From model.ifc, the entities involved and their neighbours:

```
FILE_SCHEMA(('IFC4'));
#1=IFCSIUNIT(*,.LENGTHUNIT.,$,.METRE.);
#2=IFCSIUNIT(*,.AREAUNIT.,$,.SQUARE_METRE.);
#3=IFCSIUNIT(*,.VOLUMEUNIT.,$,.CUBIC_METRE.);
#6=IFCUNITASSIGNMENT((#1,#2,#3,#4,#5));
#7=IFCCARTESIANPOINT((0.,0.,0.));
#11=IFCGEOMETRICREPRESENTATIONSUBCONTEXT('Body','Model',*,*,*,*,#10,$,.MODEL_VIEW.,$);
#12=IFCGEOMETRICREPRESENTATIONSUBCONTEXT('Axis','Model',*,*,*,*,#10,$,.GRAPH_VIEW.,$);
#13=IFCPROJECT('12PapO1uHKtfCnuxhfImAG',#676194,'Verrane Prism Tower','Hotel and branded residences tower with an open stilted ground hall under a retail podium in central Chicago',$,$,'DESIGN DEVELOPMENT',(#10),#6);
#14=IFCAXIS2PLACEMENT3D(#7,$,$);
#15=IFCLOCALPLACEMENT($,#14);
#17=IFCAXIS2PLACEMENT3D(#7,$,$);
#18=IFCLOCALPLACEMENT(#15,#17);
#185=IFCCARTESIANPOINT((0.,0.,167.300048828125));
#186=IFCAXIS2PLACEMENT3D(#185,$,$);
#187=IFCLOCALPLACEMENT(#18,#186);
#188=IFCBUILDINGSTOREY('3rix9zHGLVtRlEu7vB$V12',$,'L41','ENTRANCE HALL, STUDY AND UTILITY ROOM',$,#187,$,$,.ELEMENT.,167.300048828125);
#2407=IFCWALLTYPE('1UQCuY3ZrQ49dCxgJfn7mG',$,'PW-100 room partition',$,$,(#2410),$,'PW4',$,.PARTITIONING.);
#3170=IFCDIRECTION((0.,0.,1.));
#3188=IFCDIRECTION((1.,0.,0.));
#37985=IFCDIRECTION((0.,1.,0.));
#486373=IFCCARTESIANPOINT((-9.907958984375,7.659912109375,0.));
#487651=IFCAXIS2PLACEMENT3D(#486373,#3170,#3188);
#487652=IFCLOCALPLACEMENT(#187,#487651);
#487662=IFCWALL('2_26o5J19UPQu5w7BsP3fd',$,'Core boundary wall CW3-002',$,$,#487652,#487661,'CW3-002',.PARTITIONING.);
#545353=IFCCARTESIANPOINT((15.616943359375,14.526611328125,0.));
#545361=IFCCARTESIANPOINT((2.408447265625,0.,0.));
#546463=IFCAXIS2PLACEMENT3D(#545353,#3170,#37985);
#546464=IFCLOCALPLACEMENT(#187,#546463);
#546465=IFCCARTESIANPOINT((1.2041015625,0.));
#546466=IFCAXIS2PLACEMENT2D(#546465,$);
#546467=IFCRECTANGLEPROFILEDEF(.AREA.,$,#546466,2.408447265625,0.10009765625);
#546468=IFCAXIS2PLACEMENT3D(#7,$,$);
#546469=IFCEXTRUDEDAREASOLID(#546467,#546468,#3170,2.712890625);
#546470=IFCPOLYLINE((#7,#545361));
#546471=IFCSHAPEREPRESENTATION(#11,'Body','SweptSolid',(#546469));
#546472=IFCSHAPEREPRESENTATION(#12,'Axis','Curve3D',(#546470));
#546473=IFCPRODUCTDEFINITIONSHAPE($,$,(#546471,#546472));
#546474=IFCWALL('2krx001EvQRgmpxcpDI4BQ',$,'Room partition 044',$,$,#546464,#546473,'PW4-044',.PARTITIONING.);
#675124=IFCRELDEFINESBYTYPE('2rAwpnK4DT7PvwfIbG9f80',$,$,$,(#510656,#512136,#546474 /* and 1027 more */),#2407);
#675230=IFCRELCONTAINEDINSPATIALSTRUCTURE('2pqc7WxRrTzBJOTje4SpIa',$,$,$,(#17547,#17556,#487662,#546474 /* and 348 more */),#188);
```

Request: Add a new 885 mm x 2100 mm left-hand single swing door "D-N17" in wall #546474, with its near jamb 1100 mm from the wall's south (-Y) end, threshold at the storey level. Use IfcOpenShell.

```python
import numpy as np
import ifcopenshell
import ifcopenshell.api.feature
import ifcopenshell.api.geometry
import ifcopenshell.api.root
import ifcopenshell.api.spatial
import ifcopenshell.geom
import ifcopenshell.util.element
import ifcopenshell.util.placement
import ifcopenshell.util.representation
import ifcopenshell.util.shape
import ifcopenshell.util.unit

model = ifcopenshell.open("model.ifc")
unit_scale = ifcopenshell.util.unit.calculate_unit_scale(model)
settings = ifcopenshell.geom.settings()


def volume(element):
    """Net volume in cubic metres, openings subtracted."""
    shape = ifcopenshell.geom.create_shape(settings, element)
    return ifcopenshell.util.shape.get_volume(shape.geometry)


wall = model.by_guid("2krx001EvQRgmpxcpDI4BQ")
storey = ifcopenshell.util.element.get_container(wall, ifc_class="IfcBuildingStorey")
context = ifcopenshell.util.representation.get_context(model, "Model", "Body", "MODEL_VIEW")
before = volume(wall)

width, height, from_end, sill = 0.885, 2.1, 1.1, 0.0  # metres

# The wall runs along its own X axis, and the end named is its -X end.
wall_shape = ifcopenshell.geom.create_shape(settings, wall)
x, y, z = ifcopenshell.util.shape.get_vertices(wall_shape.geometry).T
start = x.min() + from_end
face, thickness = float(y.min()), float(y.max() - y.min())
wall_matrix = ifcopenshell.util.placement.get_local_placement(wall.ObjectPlacement)
level = ifcopenshell.util.placement.get_local_placement(storey.ObjectPlacement)[2, 3]


def in_wall(x, y):
    """Placement at x, y metres in the wall's axes, at sill height."""
    matrix = wall_matrix.copy()
    matrix[:, 3] = wall_matrix @ np.array([x / unit_scale, y / unit_scale, 0.0, 1.0])
    matrix[2, 3] = level + sill / unit_scale
    return matrix


# Opening: a box that overshoots both wall faces by 50 mm.
opening = ifcopenshell.api.root.create_entity(model, ifc_class="IfcOpeningElement", predefined_type="OPENING")
box = ifcopenshell.api.geometry.add_wall_representation(
    model, context=context, length=width, height=height, thickness=thickness + 0.1
)
ifcopenshell.api.geometry.assign_representation(model, product=opening, representation=box)
ifcopenshell.api.geometry.edit_object_placement(model, product=opening, matrix=in_wall(start, face - 0.05), is_si=False)
ifcopenshell.api.feature.add_feature(model, feature=opening, element=wall)

door = ifcopenshell.api.root.create_entity(model, ifc_class="IfcDoor", name="D-N17", predefined_type="DOOR")
door.OverallWidth, door.OverallHeight = width / unit_scale, height / unit_scale
door.OperationType = "SINGLE_SWING_LEFT"
body = ifcopenshell.api.geometry.add_door_representation(
    model,
    context=context,
    overall_width=door.OverallWidth,
    overall_height=door.OverallHeight,
    operation_type="SINGLE_SWING_LEFT",
    lining_properties={"LiningDepth": thickness / unit_scale, "ThresholdDepth": thickness / unit_scale},
)
ifcopenshell.api.geometry.assign_representation(model, product=door, representation=body)
ifcopenshell.api.spatial.assign_container(model, products=[door], relating_structure=storey)
ifcopenshell.api.feature.add_filling(model, opening=opening, element=door)

# The lining spans the wall, so the door starts at the wall face.
ifcopenshell.api.geometry.edit_object_placement(model, product=door, matrix=in_wall(start, face), is_si=False)

after = volume(wall)

print(f"wall volume {before:.3f} -> {after:.3f} m3")

model.write("model-out.ifc")
```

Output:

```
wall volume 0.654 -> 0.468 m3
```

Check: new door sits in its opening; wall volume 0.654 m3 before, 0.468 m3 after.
